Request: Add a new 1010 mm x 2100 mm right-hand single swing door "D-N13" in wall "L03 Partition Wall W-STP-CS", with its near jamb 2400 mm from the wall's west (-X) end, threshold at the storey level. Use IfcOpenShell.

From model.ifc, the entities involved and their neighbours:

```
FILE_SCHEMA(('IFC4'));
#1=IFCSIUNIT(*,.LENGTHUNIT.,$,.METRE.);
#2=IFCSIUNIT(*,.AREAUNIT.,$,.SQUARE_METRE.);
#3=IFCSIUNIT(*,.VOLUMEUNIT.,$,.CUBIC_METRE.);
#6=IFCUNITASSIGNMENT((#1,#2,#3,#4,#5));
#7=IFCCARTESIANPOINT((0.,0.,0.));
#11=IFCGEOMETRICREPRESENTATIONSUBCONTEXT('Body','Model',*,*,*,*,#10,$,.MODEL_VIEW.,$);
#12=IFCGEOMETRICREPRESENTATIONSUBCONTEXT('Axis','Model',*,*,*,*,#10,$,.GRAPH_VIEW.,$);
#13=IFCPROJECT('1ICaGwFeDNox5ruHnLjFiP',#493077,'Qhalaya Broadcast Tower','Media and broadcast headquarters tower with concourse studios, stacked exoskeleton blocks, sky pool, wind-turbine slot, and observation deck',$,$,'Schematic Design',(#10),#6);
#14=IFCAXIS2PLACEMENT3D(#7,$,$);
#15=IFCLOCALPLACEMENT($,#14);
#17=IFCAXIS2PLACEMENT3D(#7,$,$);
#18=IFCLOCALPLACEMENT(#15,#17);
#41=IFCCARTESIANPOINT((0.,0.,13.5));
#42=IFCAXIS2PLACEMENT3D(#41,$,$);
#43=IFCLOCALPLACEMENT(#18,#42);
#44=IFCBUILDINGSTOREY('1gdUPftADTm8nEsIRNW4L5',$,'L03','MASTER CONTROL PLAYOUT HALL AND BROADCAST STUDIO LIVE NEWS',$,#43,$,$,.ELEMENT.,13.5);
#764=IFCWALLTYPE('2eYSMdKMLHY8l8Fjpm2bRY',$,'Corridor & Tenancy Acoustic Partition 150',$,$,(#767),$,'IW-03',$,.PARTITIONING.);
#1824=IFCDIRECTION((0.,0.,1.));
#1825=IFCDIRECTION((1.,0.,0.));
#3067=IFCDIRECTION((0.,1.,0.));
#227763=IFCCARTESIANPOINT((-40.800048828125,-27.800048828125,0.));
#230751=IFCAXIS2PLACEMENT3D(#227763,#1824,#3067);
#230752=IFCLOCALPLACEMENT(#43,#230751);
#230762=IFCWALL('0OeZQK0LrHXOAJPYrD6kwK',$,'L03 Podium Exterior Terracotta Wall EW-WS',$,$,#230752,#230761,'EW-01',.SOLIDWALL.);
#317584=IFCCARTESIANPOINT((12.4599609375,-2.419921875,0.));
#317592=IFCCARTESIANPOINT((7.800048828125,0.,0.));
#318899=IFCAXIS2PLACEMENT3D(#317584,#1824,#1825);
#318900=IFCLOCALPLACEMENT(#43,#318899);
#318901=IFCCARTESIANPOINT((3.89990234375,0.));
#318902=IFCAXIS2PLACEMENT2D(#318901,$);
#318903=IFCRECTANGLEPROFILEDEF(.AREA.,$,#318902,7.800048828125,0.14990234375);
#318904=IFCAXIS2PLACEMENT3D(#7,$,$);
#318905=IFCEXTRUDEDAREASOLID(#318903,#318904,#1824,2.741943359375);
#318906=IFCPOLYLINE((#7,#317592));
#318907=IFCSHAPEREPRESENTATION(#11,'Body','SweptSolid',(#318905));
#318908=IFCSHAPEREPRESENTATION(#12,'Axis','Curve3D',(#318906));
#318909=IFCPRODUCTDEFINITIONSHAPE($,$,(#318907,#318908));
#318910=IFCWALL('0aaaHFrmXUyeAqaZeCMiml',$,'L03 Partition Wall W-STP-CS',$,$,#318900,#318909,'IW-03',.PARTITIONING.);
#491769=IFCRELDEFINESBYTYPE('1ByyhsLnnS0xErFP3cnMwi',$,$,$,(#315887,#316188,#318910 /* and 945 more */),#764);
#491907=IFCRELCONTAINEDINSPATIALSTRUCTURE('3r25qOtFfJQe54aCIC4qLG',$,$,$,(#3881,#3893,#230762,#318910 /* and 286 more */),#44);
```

```python
import numpy as np
import ifcopenshell
import ifcopenshell.api.feature
import ifcopenshell.api.geometry
import ifcopenshell.api.root
import ifcopenshell.api.spatial
import ifcopenshell.geom
import ifcopenshell.util.element
import ifcopenshell.util.placement
import ifcopenshell.util.representation
import ifcopenshell.util.shape
import ifcopenshell.util.unit

model = ifcopenshell.open("model.ifc")
unit_scale = ifcopenshell.util.unit.calculate_unit_scale(model)
settings = ifcopenshell.geom.settings()


def volume(element):
    """Net volume in cubic metres, openings subtracted."""
    shape = ifcopenshell.geom.create_shape(settings, element)
    return ifcopenshell.util.shape.get_volume(shape.geometry)


wall = model.by_guid("0aaaHFrmXUyeAqaZeCMiml")
storey = ifcopenshell.util.element.get_container(wall, ifc_class="IfcBuildingStorey")
context = ifcopenshell.util.representation.get_context(model, "Model", "Body", "MODEL_VIEW")
before = volume(wall)

width, height, from_end, sill = 1.01, 2.1, 2.4, 0.0  # metres

# The wall runs along its own X axis, and the end named is its -X end.
wall_shape = ifcopenshell.geom.create_shape(settings, wall)
x, y, z = ifcopenshell.util.shape.get_vertices(wall_shape.geometry).T
start = x.min() + from_end
face, thickness = float(y.min()), float(y.max() - y.min())
wall_matrix = ifcopenshell.util.placement.get_local_placement(wall.ObjectPlacement)
level = ifcopenshell.util.placement.get_local_placement(storey.ObjectPlacement)[2, 3]


def in_wall(x, y):
    """Placement at x, y metres in the wall's axes, at sill height."""
    matrix = wall_matrix.copy()
    matrix[:, 3] = wall_matrix @ np.array([x / unit_scale, y / unit_scale, 0.0, 1.0])
    matrix[2, 3] = level + sill / unit_scale
    return matrix


# Opening: a box that overshoots both wall faces by 50 mm.
opening = ifcopenshell.api.root.create_entity(model, ifc_class="IfcOpeningElement", predefined_type="OPENING")
box = ifcopenshell.api.geometry.add_wall_representation(
    model, context=context, length=width, height=height, thickness=thickness + 0.1
)
ifcopenshell.api.geometry.assign_representation(model, product=opening, representation=box)
ifcopenshell.api.geometry.edit_object_placement(model, product=opening, matrix=in_wall(start, face - 0.05), is_si=False)
ifcopenshell.api.feature.add_feature(model, feature=opening, element=wall)

door = ifcopenshell.api.root.create_entity(model, ifc_class="IfcDoor", name="D-N13", predefined_type="DOOR")
door.OverallWidth, door.OverallHeight = width / unit_scale, height / unit_scale
door.OperationType = "SINGLE_SWING_RIGHT"
body = ifcopenshell.api.geometry.add_door_representation(
    model,
    context=context,
    overall_width=door.OverallWidth,
    overall_height=door.OverallHeight,
    operation_type="SINGLE_SWING_RIGHT",
    lining_properties={"LiningDepth": thickness / unit_scale, "ThresholdDepth": thickness / unit_scale},
)
ifcopenshell.api.geometry.assign_representation(model, product=door, representation=body)
ifcopenshell.api.spatial.assign_container(model, products=[door], relating_structure=storey)
ifcopenshell.api.feature.add_filling(model, opening=opening, element=door)

# The lining spans the wall, so the door starts at the wall face.
ifcopenshell.api.geometry.edit_object_placement(model, product=door, matrix=in_wall(start, face), is_si=False)

after = volume(wall)

print(f"wall volume {before:.3f} -> {after:.3f} m3")

model.write("model_edited.ifc")
```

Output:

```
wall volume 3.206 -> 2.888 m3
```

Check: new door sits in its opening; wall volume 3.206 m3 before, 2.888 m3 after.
